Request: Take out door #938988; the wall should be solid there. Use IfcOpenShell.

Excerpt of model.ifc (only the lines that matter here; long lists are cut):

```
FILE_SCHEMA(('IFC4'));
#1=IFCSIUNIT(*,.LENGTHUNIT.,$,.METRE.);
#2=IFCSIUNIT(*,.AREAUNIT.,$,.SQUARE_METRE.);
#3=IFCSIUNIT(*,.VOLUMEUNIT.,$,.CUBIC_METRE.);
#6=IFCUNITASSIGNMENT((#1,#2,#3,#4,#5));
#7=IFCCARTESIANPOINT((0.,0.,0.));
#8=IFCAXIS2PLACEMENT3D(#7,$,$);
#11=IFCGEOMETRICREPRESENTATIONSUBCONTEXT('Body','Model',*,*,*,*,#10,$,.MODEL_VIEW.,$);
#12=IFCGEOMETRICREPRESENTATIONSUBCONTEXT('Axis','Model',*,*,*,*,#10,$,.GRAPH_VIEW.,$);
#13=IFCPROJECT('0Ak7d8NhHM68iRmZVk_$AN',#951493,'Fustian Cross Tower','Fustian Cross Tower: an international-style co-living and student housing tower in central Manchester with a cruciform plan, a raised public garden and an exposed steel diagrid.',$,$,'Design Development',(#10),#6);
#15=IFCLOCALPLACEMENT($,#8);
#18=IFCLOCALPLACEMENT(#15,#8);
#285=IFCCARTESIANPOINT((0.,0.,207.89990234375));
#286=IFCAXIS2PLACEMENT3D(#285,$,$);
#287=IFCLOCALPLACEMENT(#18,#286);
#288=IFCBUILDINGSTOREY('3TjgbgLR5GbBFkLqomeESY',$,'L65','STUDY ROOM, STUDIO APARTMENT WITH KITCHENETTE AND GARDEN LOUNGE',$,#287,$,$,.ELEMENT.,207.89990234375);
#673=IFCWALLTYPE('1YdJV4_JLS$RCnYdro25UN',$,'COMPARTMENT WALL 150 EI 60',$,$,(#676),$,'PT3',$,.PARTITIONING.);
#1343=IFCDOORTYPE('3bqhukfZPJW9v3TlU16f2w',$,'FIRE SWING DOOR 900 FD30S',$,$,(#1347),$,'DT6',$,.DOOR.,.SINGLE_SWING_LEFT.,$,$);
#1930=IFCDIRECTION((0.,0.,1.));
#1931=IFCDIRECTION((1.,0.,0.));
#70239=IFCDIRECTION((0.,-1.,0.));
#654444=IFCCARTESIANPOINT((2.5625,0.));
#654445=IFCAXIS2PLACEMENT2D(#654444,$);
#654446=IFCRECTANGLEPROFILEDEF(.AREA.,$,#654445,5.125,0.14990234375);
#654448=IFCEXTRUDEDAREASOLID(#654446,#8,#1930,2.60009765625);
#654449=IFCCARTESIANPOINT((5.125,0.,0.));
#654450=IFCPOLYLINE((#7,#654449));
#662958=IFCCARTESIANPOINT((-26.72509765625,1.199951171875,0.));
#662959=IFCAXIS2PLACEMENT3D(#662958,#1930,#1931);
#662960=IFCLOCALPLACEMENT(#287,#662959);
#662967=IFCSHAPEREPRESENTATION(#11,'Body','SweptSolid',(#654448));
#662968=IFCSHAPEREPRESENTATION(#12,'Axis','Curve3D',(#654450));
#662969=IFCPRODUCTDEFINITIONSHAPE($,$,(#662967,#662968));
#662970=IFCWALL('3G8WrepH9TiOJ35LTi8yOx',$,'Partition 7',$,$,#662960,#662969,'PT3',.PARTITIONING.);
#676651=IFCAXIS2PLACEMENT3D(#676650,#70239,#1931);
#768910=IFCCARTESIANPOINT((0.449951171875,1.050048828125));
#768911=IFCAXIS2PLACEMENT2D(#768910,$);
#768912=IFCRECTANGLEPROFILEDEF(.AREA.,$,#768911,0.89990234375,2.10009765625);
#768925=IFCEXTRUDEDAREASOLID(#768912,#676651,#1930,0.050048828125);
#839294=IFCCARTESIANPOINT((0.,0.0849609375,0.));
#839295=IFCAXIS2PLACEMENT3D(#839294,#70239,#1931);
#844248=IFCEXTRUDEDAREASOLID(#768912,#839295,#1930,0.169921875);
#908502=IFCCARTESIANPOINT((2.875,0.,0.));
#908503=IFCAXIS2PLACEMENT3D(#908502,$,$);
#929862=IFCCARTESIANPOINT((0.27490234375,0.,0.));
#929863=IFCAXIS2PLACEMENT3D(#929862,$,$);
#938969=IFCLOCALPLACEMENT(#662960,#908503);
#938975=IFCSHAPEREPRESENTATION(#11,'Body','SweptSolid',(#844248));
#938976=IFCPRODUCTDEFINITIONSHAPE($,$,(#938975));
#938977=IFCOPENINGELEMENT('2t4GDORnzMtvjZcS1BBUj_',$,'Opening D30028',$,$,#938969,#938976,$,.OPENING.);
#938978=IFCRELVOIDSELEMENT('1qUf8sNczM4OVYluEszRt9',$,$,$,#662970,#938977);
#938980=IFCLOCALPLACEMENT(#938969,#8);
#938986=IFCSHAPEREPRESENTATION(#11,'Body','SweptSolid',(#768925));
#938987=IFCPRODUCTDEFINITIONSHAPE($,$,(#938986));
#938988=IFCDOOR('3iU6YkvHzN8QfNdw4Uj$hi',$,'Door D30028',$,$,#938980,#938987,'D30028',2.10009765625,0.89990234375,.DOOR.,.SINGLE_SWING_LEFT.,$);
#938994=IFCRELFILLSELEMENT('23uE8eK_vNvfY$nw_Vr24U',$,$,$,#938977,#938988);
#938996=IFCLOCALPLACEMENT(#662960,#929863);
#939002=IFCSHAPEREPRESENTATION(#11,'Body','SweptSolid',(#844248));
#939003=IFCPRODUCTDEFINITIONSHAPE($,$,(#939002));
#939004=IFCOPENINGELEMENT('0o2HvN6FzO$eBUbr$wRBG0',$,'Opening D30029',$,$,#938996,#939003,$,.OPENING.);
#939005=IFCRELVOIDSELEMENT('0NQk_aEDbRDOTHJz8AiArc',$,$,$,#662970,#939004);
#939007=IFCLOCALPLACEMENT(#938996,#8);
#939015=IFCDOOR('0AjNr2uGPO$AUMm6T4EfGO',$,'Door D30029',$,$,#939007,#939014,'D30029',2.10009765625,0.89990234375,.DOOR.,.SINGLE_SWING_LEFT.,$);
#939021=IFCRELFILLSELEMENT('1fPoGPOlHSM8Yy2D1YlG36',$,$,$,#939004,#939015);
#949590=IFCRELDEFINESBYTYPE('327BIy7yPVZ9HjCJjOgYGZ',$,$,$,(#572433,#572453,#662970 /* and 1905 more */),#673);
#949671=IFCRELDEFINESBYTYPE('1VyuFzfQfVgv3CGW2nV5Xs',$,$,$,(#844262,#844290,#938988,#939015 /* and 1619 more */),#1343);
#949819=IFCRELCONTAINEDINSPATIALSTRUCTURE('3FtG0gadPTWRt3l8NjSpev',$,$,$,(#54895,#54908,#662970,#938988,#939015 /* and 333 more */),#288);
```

```python
import ifcopenshell
import ifcopenshell.api.feature
import ifcopenshell.api.root
import ifcopenshell.geom
import ifcopenshell.util.shape

model = ifcopenshell.open("model.ifc")
settings = ifcopenshell.geom.settings()


def volume(element):
    """Net volume in cubic metres, openings subtracted."""
    shape = ifcopenshell.geom.create_shape(settings, element)
    return ifcopenshell.util.shape.get_volume(shape.geometry)


door = model.by_id(938988)
opening = door.FillsVoids[0].RelatingOpeningElement
wall = opening.VoidsElements[0].RelatingBuildingElement
before = volume(wall)

ifcopenshell.api.root.remove_product(model, product=door)
ifcopenshell.api.feature.remove_feature(model, feature=opening)

after = volume(wall)

print(f"wall volume {before:.3f} -> {after:.3f} m3")

model.write("model_updated.ifc")
```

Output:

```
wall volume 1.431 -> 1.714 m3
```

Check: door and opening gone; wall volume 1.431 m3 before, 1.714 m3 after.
